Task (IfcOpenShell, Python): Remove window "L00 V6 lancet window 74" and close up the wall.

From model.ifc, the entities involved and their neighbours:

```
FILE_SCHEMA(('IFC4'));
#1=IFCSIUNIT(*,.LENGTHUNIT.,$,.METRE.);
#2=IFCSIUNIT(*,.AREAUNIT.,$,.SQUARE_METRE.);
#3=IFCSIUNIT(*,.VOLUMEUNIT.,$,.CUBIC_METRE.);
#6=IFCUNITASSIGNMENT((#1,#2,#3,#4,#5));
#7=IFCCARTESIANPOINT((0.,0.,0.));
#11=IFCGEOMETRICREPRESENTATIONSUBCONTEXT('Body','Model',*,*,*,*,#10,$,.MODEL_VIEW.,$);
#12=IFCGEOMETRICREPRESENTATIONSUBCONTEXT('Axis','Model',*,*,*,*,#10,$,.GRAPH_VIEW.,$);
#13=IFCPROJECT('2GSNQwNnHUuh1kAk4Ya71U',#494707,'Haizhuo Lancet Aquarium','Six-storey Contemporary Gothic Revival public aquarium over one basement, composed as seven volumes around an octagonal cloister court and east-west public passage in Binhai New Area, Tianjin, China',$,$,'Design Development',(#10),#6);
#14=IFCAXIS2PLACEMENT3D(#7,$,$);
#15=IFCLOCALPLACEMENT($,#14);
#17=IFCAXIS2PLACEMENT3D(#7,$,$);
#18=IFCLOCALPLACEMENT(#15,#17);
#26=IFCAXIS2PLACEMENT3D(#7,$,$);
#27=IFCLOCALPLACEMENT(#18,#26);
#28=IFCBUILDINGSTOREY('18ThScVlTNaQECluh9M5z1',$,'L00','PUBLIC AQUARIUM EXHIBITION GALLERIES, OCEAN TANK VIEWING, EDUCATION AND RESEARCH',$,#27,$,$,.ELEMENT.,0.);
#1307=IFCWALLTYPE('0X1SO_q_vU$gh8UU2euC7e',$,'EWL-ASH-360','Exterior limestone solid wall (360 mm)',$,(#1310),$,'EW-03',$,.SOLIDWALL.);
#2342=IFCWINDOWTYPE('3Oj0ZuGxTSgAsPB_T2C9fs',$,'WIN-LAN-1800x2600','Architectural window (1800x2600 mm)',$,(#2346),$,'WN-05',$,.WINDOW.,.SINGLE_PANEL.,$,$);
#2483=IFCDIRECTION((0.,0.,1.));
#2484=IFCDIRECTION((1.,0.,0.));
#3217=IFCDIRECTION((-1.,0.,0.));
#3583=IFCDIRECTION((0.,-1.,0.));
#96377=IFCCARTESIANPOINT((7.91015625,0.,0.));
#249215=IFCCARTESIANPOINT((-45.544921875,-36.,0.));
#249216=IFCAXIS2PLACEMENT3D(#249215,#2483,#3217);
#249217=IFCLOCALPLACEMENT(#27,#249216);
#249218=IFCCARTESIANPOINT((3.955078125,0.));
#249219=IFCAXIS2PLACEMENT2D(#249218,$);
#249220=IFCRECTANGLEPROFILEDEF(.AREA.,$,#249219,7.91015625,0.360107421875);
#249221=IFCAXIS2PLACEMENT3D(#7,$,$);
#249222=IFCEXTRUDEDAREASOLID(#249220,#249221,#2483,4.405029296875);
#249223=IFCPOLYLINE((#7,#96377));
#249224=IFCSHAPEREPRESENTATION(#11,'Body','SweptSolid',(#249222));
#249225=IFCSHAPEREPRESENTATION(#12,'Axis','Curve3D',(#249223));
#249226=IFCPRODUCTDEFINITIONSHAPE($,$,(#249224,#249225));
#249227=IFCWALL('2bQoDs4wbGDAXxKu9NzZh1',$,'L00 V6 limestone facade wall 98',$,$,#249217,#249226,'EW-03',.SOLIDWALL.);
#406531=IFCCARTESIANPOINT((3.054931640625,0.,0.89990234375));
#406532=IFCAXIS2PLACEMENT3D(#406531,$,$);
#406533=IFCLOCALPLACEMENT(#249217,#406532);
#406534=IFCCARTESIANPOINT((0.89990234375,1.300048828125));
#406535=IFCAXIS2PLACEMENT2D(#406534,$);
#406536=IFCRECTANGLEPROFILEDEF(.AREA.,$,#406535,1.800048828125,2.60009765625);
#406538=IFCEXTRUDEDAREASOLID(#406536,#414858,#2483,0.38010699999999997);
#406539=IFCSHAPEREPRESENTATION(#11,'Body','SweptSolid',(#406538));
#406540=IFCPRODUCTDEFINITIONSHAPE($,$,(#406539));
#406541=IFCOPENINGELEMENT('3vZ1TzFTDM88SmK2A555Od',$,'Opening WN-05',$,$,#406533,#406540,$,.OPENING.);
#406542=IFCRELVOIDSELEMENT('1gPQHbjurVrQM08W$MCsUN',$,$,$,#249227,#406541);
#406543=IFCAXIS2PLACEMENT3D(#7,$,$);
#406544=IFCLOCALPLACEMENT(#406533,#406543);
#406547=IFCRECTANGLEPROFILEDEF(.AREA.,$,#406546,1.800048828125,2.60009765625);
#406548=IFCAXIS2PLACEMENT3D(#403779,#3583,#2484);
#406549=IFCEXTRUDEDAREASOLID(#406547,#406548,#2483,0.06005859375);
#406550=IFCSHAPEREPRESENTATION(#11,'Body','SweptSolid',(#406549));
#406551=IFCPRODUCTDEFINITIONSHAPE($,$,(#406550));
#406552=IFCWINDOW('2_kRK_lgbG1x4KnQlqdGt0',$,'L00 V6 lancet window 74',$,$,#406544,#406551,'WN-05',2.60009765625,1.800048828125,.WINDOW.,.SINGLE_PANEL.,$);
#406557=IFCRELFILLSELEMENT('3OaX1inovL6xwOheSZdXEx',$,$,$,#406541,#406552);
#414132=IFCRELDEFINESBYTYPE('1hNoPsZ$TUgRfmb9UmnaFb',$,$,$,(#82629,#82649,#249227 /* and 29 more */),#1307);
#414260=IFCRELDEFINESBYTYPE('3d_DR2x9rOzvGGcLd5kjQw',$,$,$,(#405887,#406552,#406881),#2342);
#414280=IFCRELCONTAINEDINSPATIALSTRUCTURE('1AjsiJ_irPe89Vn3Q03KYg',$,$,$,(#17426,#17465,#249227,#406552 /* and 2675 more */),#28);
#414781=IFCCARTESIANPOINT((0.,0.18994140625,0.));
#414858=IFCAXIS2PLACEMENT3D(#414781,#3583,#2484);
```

```python
import ifcopenshell
import ifcopenshell.api.feature
import ifcopenshell.api.root
import ifcopenshell.geom
import ifcopenshell.util.shape

model = ifcopenshell.open("model.ifc")
settings = ifcopenshell.geom.settings()


def volume(element):
    """Net volume in cubic metres, openings subtracted."""
    shape = ifcopenshell.geom.create_shape(settings, element)
    return ifcopenshell.util.shape.get_volume(shape.geometry)


window = model.by_id(406552)
opening = window.FillsVoids[0].RelatingOpeningElement
wall = opening.VoidsElements[0].RelatingBuildingElement
before = volume(wall)

ifcopenshell.api.root.remove_product(model, product=window)
ifcopenshell.api.feature.remove_feature(model, feature=opening)

after = volume(wall)

print(f"wall volume {before:.3f} -> {after:.3f} m3")

model.write("model-out.ifc")
```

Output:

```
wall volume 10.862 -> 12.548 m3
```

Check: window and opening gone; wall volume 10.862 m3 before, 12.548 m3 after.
